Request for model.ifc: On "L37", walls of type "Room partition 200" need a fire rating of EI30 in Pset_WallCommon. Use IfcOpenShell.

First a look at what the model holds.

```python
import ifcopenshell
import ifcopenshell.util.element

model = ifcopenshell.open("model.ifc")
print(model.schema)
storey = next(s for s in model.by_type("IfcBuildingStorey") if s.Name == "L37")
walls = [e for e in ifcopenshell.util.element.get_decomposition(storey) if e.is_a("IfcWall")]
seen = {}
for e in walls:
    element_type = ifcopenshell.util.element.get_type(e)
    key = (element_type.Name if element_type != e and element_type else None, ifcopenshell.util.element.get_pset(e, "Pset_WallCommon", "FireRating"))
    seen[key] = seen.get(key, 0) + 1
for (name, value), count in sorted(seen.items(), key=str):
    print(count, "x", name, "|", value)
```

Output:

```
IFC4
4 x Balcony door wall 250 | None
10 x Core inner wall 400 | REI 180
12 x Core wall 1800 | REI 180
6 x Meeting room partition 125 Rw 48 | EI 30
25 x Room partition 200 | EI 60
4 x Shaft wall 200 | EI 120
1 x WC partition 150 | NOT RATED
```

```python
import ifcopenshell
import ifcopenshell.api.pset
import ifcopenshell.util.element

model = ifcopenshell.open("model.ifc")

storey = next(s for s in model.by_type("IfcBuildingStorey") if s.Name == "L37")
walls = [e for e in ifcopenshell.util.element.get_decomposition(storey) if e.is_a("IfcWall")]

count = 0
for e in walls:
    element_type = ifcopenshell.util.element.get_type(e)
    if element_type in (None, e) or element_type.Name != "Room partition 200":
        continue
    found = ifcopenshell.util.element.get_pset(e, "Pset_WallCommon", should_inherit=False)
    if found:
        pset = model.by_id(found["id"])
        if len(ifcopenshell.util.element.get_elements_by_pset(pset)) > 1:
            pset = ifcopenshell.api.pset.unshare_pset(model, products=[e], pset=pset)[0]
    else:
        pset = ifcopenshell.api.pset.add_pset(model, product=e, name="Pset_WallCommon")
    ifcopenshell.api.pset.edit_pset(model, pset=pset, properties={"FireRating": "EI30"})
    count += 1

print(count, "walls updated")

model.write("model_updated.ifc")
```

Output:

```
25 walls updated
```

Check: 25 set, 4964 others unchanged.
